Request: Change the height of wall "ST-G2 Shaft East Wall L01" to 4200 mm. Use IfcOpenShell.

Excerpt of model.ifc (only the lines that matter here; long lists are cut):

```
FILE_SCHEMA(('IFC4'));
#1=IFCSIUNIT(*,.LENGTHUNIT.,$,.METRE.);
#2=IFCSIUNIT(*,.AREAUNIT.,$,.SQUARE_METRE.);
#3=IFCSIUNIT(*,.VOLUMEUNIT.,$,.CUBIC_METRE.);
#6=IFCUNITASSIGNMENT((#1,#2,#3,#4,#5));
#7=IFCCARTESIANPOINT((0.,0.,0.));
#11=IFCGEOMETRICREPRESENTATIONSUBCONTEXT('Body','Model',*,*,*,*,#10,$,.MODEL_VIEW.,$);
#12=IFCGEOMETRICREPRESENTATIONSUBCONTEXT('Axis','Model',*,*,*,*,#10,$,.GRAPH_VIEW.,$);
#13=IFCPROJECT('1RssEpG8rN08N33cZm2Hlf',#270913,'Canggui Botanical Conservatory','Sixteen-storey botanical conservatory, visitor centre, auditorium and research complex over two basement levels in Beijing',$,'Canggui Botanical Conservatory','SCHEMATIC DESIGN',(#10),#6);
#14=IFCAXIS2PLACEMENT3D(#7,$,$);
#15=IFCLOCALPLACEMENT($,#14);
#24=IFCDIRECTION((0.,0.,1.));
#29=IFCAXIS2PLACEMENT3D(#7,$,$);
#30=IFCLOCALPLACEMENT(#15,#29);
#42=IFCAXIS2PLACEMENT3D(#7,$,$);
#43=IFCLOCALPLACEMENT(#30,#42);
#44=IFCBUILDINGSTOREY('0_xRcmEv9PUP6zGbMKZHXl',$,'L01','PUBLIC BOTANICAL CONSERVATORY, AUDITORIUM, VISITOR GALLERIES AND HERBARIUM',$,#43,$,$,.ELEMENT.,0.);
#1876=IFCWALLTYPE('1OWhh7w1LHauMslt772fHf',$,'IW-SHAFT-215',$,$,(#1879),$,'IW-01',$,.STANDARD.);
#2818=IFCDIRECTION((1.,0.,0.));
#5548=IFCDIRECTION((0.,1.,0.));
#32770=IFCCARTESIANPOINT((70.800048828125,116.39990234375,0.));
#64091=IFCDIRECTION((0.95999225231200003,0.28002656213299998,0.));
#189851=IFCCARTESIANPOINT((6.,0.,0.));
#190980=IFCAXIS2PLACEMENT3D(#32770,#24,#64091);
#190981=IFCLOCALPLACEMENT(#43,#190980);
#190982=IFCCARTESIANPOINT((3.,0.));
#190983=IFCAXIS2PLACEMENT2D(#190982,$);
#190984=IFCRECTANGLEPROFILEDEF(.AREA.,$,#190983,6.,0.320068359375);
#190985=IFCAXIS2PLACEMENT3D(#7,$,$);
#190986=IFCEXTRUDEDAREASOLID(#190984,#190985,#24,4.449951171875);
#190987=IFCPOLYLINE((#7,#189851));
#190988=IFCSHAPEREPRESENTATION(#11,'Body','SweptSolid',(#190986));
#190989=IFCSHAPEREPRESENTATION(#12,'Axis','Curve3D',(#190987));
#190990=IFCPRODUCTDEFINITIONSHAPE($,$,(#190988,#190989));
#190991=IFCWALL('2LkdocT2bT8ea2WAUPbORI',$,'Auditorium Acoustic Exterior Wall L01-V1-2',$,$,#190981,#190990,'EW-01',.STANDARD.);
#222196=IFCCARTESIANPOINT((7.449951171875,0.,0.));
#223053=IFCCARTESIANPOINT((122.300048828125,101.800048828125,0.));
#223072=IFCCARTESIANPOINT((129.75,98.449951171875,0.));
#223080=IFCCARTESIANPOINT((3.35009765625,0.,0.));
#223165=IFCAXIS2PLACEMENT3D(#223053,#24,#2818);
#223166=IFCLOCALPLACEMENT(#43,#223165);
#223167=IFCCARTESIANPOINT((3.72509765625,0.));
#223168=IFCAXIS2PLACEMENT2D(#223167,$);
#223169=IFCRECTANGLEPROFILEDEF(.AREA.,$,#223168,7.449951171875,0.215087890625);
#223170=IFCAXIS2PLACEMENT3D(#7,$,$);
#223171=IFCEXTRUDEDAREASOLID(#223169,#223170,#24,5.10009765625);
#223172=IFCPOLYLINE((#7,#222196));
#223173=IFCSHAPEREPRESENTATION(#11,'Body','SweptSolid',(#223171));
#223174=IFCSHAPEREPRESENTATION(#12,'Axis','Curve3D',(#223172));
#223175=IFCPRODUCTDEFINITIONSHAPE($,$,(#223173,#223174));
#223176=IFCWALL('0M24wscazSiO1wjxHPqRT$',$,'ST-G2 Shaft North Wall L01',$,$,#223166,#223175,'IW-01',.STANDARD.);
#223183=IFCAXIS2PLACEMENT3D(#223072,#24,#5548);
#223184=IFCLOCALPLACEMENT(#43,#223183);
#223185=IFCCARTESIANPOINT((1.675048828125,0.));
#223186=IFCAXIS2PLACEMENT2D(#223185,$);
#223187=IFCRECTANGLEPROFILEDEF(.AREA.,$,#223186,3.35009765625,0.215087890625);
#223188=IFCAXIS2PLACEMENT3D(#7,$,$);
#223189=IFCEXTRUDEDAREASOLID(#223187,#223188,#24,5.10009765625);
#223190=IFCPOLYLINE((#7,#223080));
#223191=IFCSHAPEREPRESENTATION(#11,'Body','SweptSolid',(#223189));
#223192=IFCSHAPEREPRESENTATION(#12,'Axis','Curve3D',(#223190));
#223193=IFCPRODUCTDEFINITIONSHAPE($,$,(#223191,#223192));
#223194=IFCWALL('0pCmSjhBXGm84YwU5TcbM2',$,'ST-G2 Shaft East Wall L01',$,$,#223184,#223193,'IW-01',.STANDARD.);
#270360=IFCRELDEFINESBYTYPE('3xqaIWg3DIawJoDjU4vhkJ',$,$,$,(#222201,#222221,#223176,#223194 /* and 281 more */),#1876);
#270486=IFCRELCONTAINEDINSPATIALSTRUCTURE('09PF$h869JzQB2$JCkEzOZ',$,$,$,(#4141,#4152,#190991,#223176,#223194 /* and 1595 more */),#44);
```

```python
import ifcopenshell
import ifcopenshell.geom
import ifcopenshell.util.representation
import ifcopenshell.util.shape
import ifcopenshell.util.unit

model = ifcopenshell.open("model.ifc")
unit_scale = ifcopenshell.util.unit.calculate_unit_scale(model)
settings = ifcopenshell.geom.settings()


def volume(element):
    """Net volume in cubic metres, openings subtracted."""
    shape = ifcopenshell.geom.create_shape(settings, element)
    return ifcopenshell.util.shape.get_volume(shape.geometry)


wall = model.by_guid("0pCmSjhBXGm84YwU5TcbM2")
before = volume(wall)

body = ifcopenshell.util.representation.get_representation(wall, "Model", "Body")
solid = body.Items[0]
old_height = solid.Depth
solid.Depth = 4.2 / unit_scale
after = volume(wall)

print(f"height {old_height:g} -> {solid.Depth:g}, volume {before:.3f} -> {after:.3f} m3")

model.write("model_rev.ifc")
```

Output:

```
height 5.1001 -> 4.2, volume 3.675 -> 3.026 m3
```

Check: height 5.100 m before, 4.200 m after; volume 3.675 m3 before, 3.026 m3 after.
